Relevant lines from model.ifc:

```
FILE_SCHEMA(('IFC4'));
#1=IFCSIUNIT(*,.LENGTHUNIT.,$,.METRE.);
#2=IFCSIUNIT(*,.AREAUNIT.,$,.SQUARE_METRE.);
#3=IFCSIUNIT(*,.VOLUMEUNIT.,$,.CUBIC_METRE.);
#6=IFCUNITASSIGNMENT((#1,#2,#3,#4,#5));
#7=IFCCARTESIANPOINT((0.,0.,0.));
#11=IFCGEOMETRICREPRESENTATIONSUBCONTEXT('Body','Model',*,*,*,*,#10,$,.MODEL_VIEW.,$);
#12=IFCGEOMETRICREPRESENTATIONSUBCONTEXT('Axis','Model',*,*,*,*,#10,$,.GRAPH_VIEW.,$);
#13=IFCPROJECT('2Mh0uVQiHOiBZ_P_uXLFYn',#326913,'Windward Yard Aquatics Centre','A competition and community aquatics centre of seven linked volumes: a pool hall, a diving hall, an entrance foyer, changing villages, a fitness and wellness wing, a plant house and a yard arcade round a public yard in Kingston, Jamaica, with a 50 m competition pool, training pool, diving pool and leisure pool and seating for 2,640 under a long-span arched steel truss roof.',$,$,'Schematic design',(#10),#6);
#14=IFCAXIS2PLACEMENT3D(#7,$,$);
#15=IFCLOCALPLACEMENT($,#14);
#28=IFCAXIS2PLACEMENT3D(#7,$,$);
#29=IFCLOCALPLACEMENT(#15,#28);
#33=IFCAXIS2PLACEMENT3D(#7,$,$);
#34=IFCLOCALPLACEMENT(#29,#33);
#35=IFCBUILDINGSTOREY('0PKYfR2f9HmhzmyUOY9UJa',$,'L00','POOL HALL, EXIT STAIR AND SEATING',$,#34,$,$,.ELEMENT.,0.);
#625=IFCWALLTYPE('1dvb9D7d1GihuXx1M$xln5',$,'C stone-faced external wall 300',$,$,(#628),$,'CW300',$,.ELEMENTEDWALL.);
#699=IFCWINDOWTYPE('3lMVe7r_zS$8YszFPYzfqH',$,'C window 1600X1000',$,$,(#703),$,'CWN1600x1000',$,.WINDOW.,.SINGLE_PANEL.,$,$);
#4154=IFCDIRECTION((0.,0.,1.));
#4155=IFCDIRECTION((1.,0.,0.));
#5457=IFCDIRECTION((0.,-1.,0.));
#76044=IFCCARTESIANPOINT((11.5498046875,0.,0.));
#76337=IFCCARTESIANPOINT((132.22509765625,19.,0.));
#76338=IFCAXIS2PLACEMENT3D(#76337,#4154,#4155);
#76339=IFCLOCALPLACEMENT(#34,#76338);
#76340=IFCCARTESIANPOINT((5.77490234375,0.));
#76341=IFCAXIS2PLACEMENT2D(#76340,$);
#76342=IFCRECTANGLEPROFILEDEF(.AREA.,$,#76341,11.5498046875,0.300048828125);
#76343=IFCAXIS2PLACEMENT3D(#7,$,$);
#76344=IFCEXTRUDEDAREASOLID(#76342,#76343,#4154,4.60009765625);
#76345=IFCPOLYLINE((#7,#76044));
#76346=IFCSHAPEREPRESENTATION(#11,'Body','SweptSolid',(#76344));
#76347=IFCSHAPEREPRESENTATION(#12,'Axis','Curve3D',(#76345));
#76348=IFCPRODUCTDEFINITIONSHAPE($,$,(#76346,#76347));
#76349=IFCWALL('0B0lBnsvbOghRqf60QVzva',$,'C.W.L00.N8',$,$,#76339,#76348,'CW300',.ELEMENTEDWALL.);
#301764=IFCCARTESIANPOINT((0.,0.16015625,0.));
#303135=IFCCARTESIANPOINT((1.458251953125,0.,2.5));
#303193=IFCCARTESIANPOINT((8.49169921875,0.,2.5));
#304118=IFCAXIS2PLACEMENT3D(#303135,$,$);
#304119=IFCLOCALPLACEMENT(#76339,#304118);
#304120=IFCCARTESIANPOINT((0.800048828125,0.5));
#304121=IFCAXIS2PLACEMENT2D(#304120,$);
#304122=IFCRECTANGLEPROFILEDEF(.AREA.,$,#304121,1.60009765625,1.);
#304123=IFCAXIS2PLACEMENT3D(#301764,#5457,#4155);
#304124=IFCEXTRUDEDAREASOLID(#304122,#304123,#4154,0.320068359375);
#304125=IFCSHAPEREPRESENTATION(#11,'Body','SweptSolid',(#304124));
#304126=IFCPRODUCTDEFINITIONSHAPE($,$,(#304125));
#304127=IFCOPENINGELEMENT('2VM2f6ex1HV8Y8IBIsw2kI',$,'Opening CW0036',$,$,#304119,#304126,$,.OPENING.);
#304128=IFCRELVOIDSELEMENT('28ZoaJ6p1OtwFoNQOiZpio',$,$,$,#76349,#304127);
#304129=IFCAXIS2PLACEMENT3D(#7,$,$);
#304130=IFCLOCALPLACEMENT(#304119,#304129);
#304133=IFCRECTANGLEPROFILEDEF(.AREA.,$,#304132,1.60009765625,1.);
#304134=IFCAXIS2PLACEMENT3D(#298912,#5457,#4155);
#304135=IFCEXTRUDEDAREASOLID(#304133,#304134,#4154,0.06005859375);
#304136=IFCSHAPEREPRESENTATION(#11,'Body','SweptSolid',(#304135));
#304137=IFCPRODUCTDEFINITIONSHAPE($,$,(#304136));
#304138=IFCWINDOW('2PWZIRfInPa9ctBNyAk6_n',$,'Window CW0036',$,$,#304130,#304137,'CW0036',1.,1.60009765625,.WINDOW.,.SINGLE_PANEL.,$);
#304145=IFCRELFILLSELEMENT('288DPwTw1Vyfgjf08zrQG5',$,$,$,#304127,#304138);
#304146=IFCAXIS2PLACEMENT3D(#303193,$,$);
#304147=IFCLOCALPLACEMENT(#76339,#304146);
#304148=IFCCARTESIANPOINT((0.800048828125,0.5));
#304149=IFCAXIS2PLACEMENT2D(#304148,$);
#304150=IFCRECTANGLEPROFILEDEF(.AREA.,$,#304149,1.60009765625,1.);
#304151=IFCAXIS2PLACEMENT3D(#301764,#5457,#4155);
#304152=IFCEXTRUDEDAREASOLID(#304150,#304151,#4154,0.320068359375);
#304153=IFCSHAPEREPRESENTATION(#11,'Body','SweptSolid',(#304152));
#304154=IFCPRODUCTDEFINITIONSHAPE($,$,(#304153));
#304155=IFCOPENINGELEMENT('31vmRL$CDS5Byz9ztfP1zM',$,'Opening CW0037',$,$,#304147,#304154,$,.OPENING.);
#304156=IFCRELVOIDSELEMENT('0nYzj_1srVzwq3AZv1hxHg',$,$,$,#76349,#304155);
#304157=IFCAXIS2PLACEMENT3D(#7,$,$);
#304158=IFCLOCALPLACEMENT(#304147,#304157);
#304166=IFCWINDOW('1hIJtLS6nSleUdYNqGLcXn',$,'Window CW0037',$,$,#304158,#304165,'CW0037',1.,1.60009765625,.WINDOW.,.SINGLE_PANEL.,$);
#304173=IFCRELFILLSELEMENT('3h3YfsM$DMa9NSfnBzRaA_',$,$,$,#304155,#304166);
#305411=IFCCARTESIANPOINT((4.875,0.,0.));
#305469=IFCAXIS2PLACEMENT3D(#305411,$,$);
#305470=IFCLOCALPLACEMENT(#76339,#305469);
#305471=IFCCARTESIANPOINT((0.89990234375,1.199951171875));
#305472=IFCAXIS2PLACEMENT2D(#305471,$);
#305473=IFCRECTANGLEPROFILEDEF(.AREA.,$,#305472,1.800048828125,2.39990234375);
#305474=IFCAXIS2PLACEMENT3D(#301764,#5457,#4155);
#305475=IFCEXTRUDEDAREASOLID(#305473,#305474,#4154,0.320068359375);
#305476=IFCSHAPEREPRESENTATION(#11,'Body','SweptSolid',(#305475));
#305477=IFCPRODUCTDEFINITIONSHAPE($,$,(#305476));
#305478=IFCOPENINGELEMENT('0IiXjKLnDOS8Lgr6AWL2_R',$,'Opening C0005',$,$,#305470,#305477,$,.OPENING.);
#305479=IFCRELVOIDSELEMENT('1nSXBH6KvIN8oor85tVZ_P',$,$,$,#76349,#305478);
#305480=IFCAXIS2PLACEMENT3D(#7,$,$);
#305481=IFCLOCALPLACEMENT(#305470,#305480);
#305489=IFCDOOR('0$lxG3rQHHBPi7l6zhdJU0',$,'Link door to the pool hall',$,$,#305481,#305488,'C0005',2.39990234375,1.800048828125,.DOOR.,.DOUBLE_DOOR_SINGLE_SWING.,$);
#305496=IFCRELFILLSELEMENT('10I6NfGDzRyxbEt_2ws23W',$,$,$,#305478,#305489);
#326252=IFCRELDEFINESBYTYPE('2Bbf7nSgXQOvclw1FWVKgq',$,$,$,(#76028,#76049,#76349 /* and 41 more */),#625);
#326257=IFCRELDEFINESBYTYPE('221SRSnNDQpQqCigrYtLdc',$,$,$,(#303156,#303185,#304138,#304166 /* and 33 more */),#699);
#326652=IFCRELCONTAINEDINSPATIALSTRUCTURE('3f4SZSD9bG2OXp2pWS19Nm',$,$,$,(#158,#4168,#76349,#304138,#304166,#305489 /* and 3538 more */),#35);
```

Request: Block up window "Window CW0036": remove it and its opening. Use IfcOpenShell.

```python
import ifcopenshell
import ifcopenshell.api.feature
import ifcopenshell.api.root
import ifcopenshell.geom
import ifcopenshell.util.shape

model = ifcopenshell.open("model.ifc")
settings = ifcopenshell.geom.settings()


def volume(element):
    """Net volume in cubic metres, openings subtracted."""
    shape = ifcopenshell.geom.create_shape(settings, element)
    return ifcopenshell.util.shape.get_volume(shape.geometry)


window = model.by_guid("2PWZIRfInPa9ctBNyAk6_n")
opening = window.FillsVoids[0].RelatingOpeningElement
wall = opening.VoidsElements[0].RelatingBuildingElement
before = volume(wall)

ifcopenshell.api.root.remove_product(model, product=window)
ifcopenshell.api.feature.remove_feature(model, feature=opening)

after = volume(wall)

print(f"wall volume {before:.3f} -> {after:.3f} m3")

model.write("model_updated.ifc")
```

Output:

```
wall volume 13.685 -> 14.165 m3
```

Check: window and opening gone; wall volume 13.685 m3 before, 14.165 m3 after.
